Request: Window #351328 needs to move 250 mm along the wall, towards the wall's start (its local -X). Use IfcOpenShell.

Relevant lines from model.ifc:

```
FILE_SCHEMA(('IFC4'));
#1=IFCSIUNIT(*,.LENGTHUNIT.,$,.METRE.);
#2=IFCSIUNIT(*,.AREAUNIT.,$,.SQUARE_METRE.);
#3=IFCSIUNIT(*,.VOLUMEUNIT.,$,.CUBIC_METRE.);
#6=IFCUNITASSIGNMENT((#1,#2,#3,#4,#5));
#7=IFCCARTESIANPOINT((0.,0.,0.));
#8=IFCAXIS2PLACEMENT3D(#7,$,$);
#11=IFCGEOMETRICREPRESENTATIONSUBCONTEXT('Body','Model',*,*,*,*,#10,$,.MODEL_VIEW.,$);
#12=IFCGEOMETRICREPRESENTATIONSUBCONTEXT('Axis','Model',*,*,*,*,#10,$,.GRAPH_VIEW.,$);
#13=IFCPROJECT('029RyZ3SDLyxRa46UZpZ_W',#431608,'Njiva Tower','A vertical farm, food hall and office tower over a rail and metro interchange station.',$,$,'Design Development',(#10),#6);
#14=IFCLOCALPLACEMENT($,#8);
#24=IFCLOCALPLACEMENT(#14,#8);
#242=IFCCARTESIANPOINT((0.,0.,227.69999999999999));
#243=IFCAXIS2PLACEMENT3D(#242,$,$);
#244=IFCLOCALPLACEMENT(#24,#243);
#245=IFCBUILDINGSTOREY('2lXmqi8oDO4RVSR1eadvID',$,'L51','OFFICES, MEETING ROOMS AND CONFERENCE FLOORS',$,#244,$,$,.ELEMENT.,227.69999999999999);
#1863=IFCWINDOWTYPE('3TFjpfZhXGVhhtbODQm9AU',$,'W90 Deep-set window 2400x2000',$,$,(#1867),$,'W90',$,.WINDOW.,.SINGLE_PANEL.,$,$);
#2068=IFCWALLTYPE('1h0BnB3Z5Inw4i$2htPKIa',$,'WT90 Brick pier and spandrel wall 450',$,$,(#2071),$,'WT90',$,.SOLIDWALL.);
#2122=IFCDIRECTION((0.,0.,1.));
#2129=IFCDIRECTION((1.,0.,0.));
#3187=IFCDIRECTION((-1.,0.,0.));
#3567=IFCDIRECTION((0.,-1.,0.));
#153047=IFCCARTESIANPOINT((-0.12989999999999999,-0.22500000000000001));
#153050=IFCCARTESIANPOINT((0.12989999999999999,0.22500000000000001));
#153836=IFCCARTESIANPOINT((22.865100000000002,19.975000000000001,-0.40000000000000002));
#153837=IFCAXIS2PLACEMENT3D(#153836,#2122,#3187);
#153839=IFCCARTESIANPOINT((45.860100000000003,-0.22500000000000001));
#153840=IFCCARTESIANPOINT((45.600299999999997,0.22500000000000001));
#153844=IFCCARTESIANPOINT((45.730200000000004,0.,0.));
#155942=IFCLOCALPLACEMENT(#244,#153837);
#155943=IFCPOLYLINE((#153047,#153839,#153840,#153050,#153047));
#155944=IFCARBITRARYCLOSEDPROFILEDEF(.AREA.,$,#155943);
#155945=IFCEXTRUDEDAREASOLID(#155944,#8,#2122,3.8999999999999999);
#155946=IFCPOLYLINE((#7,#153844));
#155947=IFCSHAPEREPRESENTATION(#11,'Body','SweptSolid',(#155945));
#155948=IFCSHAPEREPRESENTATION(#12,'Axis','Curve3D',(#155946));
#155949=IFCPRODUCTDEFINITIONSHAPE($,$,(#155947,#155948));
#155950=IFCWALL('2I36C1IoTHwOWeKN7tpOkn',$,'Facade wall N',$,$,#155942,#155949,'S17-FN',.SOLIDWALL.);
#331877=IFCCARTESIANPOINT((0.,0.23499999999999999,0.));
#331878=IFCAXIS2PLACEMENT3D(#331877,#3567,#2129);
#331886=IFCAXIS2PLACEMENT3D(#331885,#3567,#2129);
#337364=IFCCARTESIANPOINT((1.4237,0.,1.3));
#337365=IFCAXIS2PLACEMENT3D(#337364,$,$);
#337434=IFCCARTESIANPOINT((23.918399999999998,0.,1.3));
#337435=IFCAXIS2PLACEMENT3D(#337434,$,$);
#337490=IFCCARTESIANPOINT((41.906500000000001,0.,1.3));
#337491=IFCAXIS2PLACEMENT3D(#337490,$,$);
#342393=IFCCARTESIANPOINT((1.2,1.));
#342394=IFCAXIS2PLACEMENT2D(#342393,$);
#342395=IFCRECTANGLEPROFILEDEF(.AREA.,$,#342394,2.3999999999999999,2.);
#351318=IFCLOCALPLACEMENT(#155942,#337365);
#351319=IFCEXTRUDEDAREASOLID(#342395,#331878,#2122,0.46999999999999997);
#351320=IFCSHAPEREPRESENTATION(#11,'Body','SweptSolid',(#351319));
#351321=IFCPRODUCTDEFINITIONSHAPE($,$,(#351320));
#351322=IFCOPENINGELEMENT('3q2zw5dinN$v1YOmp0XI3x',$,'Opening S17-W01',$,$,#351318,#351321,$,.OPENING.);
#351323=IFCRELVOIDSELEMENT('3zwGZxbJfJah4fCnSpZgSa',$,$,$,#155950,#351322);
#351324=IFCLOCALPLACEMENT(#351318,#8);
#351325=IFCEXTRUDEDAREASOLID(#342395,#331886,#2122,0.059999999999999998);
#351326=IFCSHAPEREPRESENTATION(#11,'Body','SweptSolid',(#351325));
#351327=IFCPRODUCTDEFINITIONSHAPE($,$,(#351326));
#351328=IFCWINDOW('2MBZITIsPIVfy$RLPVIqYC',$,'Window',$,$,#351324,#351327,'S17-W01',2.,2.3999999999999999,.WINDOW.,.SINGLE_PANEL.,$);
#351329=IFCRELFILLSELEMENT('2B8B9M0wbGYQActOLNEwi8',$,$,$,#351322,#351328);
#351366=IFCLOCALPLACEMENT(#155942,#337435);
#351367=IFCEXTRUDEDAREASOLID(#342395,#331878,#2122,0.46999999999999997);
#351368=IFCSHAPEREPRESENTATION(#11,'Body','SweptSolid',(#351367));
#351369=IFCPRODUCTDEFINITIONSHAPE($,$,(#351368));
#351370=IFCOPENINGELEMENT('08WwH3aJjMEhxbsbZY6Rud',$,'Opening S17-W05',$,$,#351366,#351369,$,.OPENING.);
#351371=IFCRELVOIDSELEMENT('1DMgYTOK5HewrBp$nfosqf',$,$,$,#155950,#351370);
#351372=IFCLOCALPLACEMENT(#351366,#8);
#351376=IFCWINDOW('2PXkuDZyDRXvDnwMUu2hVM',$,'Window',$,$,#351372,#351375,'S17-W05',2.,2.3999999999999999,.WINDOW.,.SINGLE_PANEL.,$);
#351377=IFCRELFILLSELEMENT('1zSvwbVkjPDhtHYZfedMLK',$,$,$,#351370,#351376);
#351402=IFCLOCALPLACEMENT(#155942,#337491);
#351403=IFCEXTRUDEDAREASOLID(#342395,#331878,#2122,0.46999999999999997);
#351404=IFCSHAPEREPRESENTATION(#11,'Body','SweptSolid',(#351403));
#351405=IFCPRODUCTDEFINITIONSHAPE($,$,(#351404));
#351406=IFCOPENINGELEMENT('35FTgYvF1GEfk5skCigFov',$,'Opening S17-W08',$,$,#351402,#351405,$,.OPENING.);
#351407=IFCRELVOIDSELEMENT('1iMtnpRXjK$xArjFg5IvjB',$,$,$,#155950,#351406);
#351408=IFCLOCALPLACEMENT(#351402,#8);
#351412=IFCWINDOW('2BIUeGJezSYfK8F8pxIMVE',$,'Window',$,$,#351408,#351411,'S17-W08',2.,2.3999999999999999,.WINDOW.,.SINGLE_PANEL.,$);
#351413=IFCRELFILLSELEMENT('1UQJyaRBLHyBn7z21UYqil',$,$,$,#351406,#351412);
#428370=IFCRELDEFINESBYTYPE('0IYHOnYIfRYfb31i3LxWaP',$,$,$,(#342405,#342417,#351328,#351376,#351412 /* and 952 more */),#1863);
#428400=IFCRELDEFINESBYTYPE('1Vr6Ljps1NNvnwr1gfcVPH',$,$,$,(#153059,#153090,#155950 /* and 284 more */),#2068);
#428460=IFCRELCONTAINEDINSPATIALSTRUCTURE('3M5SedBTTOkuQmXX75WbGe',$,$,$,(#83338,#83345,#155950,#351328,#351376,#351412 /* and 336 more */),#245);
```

```python
import ifcopenshell
import ifcopenshell.api.geometry
import ifcopenshell.util.placement

model = ifcopenshell.open("model.ifc")

window = model.by_guid("2MBZITIsPIVfy$RLPVIqYC")
opening = window.FillsVoids[0].RelatingOpeningElement
wall = opening.VoidsElements[0].RelatingBuildingElement

wall_matrix = ifcopenshell.util.placement.get_local_placement(wall.ObjectPlacement)
shift = wall_matrix[:3, 0] * -0.25
before = ifcopenshell.util.placement.get_local_placement(window.ObjectPlacement)[:3, 3].copy()

# The window is placed relative to its opening, so it follows when the opening moves.
matrix = ifcopenshell.util.placement.get_local_placement(opening.ObjectPlacement)
matrix[:3, 3] += shift
ifcopenshell.api.geometry.edit_object_placement(
    model, product=opening, matrix=matrix, is_si=False, should_transform_children=True
)

after = ifcopenshell.util.placement.get_local_placement(window.ObjectPlacement)[:3, 3]
print("window moved by", (after - before).round(3) + 0.0)

model.write("model_updated.ifc")
```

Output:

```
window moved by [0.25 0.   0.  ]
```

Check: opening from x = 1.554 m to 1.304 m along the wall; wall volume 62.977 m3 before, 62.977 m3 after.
